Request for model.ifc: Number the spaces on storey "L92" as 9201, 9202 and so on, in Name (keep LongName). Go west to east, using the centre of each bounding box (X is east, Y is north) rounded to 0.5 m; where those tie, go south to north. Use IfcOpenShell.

First a look at what the model holds.

```python
import ifcopenshell
import ifcopenshell.util.element
import ifcopenshell.util.placement

model = ifcopenshell.open("model.ifc")
print(model.schema)
storey = next(s for s in model.by_type("IfcBuildingStorey") if s.Name == "L92")
spaces = [e for e in ifcopenshell.util.element.get_decomposition(storey) if e.is_a("IfcSpace")]
for e in sorted(spaces, key=lambda e: e.id()):
    origin = ifcopenshell.util.placement.get_local_placement(e.ObjectPlacement)[:3, 3]
    print(e.id(), e.Name, e.LongName, origin.round(2) + 0.0, sep=" | ")
```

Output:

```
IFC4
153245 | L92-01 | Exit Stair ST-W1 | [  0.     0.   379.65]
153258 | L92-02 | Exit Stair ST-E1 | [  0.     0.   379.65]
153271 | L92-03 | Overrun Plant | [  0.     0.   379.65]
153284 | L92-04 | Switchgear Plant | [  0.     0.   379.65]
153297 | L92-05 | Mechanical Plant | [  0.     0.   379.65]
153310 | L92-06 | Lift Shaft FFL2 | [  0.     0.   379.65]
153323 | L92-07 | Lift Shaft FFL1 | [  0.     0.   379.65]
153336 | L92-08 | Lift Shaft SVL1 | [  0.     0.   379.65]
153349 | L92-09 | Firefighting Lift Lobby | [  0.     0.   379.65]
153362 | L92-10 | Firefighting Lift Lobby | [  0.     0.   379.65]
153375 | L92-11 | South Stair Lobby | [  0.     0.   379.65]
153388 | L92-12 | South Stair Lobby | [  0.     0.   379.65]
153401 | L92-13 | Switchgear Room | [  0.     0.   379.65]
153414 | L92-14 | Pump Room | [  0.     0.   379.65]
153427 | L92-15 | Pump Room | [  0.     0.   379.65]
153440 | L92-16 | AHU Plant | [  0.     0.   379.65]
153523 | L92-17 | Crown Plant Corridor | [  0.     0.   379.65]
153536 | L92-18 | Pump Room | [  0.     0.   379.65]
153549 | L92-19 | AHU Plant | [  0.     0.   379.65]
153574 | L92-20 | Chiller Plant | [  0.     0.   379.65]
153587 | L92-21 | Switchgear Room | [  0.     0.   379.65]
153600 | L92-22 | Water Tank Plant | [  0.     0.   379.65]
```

```python
import ifcopenshell
import ifcopenshell.geom
import ifcopenshell.util.element
import ifcopenshell.util.shape

model = ifcopenshell.open("model.ifc")
settings = ifcopenshell.geom.settings()
settings.set("use-world-coords", True)


def centre(element):
    shape = ifcopenshell.geom.create_shape(settings, element)
    return ifcopenshell.util.shape.get_bbox_centroid(shape.geometry)


storey = next(s for s in model.by_type("IfcBuildingStorey") if s.Name == "L92")
spaces = [e for e in ifcopenshell.util.element.get_decomposition(storey) if e.is_a("IfcSpace")]

# Insertion points can sit at a corner or the storey origin, so sort by the geometry (in metres).
centres = {e: centre(e) for e in spaces}
spaces.sort(key=lambda e: (round(centres[e][0] / 0.5), centres[e][1]))

for i, e in enumerate(spaces, start=1):
    number = f"92{i:02d}"
    e.Name = number
    print(e.id(), number)

model.write("model_updated.ifc")
```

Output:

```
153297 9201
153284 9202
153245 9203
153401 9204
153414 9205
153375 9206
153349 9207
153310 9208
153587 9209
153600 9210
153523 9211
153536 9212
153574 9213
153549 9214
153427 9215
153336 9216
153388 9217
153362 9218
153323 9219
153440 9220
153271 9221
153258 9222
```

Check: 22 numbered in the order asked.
